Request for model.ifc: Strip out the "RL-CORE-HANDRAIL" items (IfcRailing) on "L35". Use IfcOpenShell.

First a look at what the model holds.

```python
import ifcopenshell
import ifcopenshell.util.element

model = ifcopenshell.open("model.ifc")
print(model.schema)
storey = next(s for s in model.by_type("IfcBuildingStorey") if s.Name == "L35")
railings = [e for e in ifcopenshell.util.element.get_decomposition(storey) if e.is_a("IfcRailing")]
seen = {}
for e in railings:
    element_type = ifcopenshell.util.element.get_type(e)
    name = element_type.Name if element_type not in (None, e) else None
    seen[name] = seen.get(name, 0) + 1
for name, count in sorted(seen.items(), key=str):
    print(count, "x", name)
```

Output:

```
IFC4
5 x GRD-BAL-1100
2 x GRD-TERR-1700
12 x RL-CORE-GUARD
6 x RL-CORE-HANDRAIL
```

```python
import ifcopenshell
import ifcopenshell.api.root
import ifcopenshell.util.element

model = ifcopenshell.open("model.ifc")

storey = next(s for s in model.by_type("IfcBuildingStorey") if s.Name == "L35")
railings = [e for e in ifcopenshell.util.element.get_decomposition(storey) if e.is_a("IfcRailing")]
targets = [e for e in railings if (t := ifcopenshell.util.element.get_type(e)) not in (None, e) and t.Name == "RL-CORE-HANDRAIL"]

for e in targets:
    ifcopenshell.api.root.remove_product(model, product=e)
print(len(targets), "removed")

model.write("model-out.ifc")
```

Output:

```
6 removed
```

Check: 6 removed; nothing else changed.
